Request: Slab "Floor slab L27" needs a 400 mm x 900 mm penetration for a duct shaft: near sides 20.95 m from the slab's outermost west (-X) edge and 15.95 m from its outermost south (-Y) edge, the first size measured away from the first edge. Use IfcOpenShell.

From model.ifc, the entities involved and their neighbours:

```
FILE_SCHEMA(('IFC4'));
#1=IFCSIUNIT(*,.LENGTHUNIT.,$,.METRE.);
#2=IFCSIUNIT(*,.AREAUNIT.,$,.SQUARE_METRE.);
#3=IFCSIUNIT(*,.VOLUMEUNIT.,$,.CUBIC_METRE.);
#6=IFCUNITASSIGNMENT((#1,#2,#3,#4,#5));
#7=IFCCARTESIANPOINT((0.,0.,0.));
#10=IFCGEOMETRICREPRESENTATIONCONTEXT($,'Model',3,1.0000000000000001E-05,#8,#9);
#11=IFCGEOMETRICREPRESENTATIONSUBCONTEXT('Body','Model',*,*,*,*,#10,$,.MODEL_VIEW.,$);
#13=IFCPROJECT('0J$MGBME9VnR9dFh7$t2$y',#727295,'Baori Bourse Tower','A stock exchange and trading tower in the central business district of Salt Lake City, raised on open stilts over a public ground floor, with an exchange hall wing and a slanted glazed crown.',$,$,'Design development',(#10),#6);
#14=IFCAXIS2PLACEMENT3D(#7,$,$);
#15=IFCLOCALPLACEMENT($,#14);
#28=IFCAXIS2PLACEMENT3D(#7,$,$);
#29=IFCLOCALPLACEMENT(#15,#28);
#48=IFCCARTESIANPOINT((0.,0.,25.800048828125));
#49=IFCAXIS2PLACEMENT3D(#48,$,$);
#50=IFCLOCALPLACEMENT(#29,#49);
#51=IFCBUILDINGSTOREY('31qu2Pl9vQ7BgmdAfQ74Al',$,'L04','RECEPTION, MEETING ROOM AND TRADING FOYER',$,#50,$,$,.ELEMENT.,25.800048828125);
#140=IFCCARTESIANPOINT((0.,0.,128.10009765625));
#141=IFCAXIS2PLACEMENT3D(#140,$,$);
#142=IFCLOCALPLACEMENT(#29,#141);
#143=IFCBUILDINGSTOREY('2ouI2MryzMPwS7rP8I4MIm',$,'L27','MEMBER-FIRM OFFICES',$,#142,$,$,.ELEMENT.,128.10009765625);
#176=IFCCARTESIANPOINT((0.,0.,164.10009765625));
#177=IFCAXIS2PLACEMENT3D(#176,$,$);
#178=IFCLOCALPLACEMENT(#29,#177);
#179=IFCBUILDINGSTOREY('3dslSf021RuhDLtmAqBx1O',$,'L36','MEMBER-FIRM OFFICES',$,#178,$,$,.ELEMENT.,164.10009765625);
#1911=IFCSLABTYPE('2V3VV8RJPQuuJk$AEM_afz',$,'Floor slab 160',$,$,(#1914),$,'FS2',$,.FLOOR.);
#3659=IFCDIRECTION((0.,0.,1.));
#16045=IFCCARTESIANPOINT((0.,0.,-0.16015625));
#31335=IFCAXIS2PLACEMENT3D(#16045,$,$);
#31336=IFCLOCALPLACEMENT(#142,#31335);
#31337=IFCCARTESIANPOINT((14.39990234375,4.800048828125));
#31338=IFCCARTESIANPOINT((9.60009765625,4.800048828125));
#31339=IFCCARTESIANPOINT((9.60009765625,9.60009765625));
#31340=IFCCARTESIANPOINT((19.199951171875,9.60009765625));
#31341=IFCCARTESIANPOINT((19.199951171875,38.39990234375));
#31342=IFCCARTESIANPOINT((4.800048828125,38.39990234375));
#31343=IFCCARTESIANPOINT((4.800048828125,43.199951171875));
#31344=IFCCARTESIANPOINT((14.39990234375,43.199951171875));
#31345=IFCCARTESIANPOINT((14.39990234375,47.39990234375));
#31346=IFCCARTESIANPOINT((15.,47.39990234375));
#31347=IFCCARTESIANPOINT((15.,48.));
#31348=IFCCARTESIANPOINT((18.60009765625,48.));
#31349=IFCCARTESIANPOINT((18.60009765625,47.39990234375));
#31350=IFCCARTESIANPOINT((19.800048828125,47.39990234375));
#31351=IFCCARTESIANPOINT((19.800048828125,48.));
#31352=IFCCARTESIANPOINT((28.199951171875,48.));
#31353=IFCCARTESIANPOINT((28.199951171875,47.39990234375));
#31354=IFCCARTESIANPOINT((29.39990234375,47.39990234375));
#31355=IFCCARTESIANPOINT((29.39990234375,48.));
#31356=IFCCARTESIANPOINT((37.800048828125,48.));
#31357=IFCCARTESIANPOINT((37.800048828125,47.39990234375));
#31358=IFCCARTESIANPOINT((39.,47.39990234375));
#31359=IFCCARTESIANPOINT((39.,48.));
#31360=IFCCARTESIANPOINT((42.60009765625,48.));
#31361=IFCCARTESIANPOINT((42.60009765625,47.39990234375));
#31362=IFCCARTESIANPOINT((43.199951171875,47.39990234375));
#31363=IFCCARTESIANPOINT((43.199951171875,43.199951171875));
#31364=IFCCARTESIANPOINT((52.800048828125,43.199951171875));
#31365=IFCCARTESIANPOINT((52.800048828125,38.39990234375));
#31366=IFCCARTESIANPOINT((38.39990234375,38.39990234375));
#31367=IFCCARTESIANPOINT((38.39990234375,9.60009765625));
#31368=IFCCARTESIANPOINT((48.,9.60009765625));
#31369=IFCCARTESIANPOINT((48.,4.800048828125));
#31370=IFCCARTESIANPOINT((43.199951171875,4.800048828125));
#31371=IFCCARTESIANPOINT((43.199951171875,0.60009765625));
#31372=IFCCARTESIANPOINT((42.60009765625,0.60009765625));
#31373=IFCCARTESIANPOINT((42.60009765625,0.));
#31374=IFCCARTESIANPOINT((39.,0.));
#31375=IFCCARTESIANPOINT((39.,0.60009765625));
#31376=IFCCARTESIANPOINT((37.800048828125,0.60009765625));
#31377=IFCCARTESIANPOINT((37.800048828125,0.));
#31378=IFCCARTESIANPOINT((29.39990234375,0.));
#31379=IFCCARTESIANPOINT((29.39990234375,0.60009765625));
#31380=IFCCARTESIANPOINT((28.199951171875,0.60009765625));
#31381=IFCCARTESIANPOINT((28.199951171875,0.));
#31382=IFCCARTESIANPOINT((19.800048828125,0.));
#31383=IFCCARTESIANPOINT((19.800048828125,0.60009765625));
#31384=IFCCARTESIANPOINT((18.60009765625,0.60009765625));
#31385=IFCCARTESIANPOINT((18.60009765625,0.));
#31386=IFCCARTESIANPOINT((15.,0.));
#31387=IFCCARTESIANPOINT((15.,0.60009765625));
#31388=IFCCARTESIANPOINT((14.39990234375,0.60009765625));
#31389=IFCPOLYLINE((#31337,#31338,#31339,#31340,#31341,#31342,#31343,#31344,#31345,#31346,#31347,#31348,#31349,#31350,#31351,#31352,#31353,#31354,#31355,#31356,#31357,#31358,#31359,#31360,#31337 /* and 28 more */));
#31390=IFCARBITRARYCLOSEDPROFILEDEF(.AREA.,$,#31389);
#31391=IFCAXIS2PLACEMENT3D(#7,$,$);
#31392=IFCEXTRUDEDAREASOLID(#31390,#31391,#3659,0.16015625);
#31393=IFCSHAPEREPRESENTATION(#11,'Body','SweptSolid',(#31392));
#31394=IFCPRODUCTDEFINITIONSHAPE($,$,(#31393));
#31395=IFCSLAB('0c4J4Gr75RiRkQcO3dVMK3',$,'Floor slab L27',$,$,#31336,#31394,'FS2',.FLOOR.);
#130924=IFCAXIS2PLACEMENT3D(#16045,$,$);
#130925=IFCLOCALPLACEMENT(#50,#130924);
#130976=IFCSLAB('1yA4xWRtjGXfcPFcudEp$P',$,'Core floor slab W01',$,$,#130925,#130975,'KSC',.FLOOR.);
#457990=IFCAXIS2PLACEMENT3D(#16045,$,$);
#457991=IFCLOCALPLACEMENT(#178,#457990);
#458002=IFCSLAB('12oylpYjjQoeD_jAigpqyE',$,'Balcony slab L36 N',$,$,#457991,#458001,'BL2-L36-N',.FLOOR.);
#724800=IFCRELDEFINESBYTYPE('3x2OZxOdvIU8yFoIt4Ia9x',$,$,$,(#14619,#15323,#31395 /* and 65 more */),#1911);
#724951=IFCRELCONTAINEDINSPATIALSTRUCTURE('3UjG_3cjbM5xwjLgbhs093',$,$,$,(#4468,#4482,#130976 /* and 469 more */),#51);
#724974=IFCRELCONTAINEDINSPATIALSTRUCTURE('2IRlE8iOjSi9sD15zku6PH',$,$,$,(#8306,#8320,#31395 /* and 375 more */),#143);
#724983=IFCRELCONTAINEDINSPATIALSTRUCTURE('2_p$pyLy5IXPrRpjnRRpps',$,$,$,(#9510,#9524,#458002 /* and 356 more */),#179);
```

```python
import numpy as np
import ifcopenshell
import ifcopenshell.api.feature
import ifcopenshell.api.geometry
import ifcopenshell.api.root
import ifcopenshell.geom
import ifcopenshell.util.placement
import ifcopenshell.util.representation
import ifcopenshell.util.shape
import ifcopenshell.util.unit

model = ifcopenshell.open("model.ifc")
unit_scale = ifcopenshell.util.unit.calculate_unit_scale(model)
settings = ifcopenshell.geom.settings()


def volume(element):
    """Net volume in cubic metres, openings subtracted."""
    shape = ifcopenshell.geom.create_shape(settings, element)
    return ifcopenshell.util.shape.get_volume(shape.geometry)


slab = model.by_guid("0c4J4Gr75RiRkQcO3dVMK3")
before = volume(slab)

# Extent in the slab's own axes, in metres. The edges named are its -X and -Y sides.
slab_shape = ifcopenshell.geom.create_shape(settings, slab)
vertices = ifcopenshell.util.shape.get_vertices(slab_shape.geometry)
x_min, y_min, bottom = vertices.min(axis=0)
top = vertices[:, 2].max()

opening = ifcopenshell.api.root.create_entity(model, ifc_class="IfcOpeningElement", name="Duct shaft opening", predefined_type="OPENING")
context = ifcopenshell.util.representation.get_context(model, "Model", "Body", "MODEL_VIEW")
width, depth = 0.4, 0.9
outline = [(0.0, 0.0), (width, 0.0), (width, depth), (0.0, depth), (0.0, 0.0)]
# Overshoot both faces by 50 mm so the cut is clean.
shape = ifcopenshell.api.geometry.add_slab_representation(
    model, context=context, depth=top - bottom + 0.1, polyline=outline
)
ifcopenshell.api.geometry.assign_representation(model, product=opening, representation=shape)

matrix = ifcopenshell.util.placement.get_local_placement(slab.ObjectPlacement)
matrix[:, 3] = matrix @ np.append(np.array([x_min + 20.95, y_min + 15.95, bottom - 0.05]) / unit_scale, 1.0)
ifcopenshell.api.geometry.edit_object_placement(model, product=opening, matrix=matrix, is_si=False)
ifcopenshell.api.feature.add_feature(model, feature=opening, element=slab)

after = volume(slab)

print(f"slab volume {before:.3f} -> {after:.3f} m3")

model.write("model_edited.ifc")
```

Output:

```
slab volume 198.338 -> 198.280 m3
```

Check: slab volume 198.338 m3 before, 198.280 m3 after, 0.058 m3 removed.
